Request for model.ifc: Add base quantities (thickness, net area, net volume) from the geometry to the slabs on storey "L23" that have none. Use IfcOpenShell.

First a look at what the model holds.

```python
import ifcopenshell
import ifcopenshell.util.element
import ifcopenshell.util.unit

model = ifcopenshell.open("model.ifc")
print(model.schema)
for unit_type in ("LENGTHUNIT", "AREAUNIT", "VOLUMEUNIT"):
    print(unit_type, ifcopenshell.util.unit.calculate_unit_scale(model, unit_type))
storey = next(s for s in model.by_type("IfcBuildingStorey") if s.Name == "L23")
slabs = [e for e in ifcopenshell.util.element.get_decomposition(storey) if e.is_a("IfcSlab")]
for e in sorted(slabs, key=lambda e: e.id()):
    print(e.id(), e.is_a(), e.Name, list(ifcopenshell.util.element.get_psets(e, qtos_only=True)), sep=" | ")
```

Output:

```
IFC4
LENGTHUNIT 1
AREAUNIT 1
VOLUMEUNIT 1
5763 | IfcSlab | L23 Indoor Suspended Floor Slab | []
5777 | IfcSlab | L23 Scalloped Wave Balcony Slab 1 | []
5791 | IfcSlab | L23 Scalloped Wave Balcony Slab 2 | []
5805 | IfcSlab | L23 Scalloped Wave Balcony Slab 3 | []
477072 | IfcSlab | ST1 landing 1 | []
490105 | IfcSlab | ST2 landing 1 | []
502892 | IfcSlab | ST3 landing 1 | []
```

```python
import ifcopenshell
import ifcopenshell.api.pset
import ifcopenshell.geom
import ifcopenshell.util.element
import ifcopenshell.util.shape
import ifcopenshell.util.unit

model = ifcopenshell.open("model.ifc")
unit_scale = ifcopenshell.util.unit.calculate_unit_scale(model)
area_scale = ifcopenshell.util.unit.calculate_unit_scale(model, "AREAUNIT")
volume_scale = ifcopenshell.util.unit.calculate_unit_scale(model, "VOLUMEUNIT")
settings = ifcopenshell.geom.settings()

storey = next(s for s in model.by_type("IfcBuildingStorey") if s.Name == "L23")
slabs = [e for e in ifcopenshell.util.element.get_decomposition(storey) if e.is_a("IfcSlab")]

for e in sorted(slabs, key=lambda e: e.id()):
    if ifcopenshell.util.element.get_psets(e, qtos_only=True, should_inherit=False):
        continue
    # Geometry comes back in metres, in the element's own axes.
    shape = ifcopenshell.geom.create_shape(settings, e)
    values = {
        "Width": ifcopenshell.util.shape.get_z(shape.geometry) / unit_scale,
        "NetArea": ifcopenshell.util.shape.get_footprint_area(shape.geometry) / area_scale,
        "NetVolume": ifcopenshell.util.shape.get_volume(shape.geometry) / volume_scale,
    }
    qto = ifcopenshell.api.pset.add_qto(model, product=e, name="Qto_SlabBaseQuantities")
    ifcopenshell.api.pset.edit_qto(model, qto=qto, properties=values)
    print(e.id(), {k: round(v, 3) for k, v in values.items()})

model.write("model_rev.ifc")
```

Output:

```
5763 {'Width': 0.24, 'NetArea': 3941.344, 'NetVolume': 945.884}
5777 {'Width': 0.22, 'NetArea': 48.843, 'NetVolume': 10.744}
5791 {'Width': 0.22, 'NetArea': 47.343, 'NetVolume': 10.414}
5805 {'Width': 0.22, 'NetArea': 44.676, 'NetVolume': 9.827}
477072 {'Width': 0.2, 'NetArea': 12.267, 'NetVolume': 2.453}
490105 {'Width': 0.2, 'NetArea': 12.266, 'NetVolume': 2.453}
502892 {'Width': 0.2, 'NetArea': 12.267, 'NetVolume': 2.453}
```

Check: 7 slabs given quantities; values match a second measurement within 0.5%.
